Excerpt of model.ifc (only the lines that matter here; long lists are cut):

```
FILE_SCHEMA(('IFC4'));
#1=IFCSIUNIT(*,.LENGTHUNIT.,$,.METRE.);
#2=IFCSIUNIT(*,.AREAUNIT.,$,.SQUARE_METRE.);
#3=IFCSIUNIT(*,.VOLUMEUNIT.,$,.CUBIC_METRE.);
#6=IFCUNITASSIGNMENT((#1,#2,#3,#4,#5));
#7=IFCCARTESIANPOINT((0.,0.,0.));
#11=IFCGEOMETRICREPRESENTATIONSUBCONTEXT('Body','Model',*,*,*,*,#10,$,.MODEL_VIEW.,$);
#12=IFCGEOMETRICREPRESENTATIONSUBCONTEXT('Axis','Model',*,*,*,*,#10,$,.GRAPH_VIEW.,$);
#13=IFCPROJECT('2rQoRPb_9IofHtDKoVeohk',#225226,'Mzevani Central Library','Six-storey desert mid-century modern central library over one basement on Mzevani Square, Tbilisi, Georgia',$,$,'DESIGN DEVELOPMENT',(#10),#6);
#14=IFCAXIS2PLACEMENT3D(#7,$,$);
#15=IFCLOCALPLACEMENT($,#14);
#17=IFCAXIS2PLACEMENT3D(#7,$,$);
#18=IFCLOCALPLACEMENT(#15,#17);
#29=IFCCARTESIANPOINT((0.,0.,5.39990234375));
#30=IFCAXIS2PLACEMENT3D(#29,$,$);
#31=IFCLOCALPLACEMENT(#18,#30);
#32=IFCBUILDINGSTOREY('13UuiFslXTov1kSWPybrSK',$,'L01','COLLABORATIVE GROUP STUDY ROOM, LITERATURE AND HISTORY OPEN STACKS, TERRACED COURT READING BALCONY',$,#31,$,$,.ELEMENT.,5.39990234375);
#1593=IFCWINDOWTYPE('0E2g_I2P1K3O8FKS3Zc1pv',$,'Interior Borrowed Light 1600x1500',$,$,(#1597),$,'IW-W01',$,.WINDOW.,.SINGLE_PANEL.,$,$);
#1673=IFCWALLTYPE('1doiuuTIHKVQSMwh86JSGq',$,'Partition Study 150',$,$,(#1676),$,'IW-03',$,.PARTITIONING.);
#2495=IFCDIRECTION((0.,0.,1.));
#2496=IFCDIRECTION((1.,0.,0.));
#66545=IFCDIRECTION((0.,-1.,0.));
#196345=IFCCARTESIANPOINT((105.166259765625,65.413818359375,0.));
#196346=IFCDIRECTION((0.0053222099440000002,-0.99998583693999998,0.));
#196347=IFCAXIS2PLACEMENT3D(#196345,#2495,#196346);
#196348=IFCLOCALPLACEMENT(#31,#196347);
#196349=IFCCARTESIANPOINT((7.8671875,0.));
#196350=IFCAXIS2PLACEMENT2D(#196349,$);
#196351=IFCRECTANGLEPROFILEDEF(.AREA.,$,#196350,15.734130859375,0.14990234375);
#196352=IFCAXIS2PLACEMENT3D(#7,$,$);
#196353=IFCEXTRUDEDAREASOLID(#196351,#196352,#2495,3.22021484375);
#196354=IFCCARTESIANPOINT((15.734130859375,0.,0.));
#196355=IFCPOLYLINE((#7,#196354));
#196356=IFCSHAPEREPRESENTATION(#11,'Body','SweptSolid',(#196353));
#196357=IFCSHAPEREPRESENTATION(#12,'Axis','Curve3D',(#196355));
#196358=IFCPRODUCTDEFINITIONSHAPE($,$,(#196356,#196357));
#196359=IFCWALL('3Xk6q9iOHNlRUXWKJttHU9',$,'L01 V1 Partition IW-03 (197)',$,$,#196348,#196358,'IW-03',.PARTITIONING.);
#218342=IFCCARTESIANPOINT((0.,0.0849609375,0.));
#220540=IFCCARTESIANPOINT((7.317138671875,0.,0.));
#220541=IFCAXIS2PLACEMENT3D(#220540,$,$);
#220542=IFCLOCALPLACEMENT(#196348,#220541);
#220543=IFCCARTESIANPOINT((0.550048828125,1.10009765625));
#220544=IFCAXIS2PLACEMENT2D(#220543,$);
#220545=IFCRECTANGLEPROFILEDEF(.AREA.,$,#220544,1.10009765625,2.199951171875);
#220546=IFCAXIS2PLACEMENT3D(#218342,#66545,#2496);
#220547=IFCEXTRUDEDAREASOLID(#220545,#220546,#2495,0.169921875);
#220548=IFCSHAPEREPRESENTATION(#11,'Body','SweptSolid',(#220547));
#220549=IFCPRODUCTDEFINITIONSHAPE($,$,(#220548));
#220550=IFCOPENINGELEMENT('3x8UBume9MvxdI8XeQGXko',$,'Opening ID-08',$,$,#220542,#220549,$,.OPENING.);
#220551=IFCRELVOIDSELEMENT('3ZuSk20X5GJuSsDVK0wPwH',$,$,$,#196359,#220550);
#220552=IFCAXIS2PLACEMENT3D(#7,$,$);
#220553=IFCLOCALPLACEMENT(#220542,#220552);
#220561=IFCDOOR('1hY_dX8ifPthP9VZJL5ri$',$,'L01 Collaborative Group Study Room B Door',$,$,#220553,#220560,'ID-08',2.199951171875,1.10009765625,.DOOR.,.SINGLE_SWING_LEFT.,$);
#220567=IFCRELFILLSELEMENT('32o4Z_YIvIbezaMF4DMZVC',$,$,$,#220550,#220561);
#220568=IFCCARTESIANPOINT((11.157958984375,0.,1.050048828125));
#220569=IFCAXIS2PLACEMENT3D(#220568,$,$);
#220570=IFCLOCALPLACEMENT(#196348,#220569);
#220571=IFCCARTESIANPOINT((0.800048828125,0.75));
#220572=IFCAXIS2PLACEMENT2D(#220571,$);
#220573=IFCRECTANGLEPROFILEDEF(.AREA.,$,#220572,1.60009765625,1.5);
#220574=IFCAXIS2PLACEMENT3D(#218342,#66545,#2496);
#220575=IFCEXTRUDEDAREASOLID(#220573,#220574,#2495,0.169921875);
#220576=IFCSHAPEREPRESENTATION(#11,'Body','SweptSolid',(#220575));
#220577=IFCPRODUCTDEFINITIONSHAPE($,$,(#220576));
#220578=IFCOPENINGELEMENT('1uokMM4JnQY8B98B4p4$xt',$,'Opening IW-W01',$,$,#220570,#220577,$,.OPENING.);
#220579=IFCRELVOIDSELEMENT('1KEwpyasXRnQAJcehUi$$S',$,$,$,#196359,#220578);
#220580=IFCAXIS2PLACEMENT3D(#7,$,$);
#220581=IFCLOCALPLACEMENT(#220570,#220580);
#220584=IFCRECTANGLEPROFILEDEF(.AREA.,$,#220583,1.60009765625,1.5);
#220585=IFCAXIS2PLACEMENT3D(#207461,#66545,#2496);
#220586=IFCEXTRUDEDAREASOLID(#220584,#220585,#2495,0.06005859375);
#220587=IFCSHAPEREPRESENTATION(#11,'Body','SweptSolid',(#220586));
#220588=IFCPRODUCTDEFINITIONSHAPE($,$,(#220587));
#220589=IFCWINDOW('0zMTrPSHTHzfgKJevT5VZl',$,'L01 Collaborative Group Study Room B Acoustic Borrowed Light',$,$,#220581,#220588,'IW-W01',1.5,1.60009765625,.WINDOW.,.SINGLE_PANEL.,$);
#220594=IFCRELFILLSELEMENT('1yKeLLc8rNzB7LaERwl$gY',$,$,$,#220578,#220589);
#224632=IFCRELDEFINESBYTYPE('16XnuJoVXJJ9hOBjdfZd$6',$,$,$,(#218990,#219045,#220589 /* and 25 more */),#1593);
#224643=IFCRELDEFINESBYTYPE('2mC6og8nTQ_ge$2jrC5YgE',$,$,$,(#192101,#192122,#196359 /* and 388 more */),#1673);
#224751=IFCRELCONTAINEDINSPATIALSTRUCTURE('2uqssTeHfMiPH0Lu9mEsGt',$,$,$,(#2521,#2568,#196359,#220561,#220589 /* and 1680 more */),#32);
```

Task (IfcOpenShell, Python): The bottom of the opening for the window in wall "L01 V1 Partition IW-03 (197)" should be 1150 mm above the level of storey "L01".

```python
import numpy as np
import ifcopenshell
import ifcopenshell.api.geometry
import ifcopenshell.geom
import ifcopenshell.util.element
import ifcopenshell.util.placement
import ifcopenshell.util.shape
import ifcopenshell.util.unit

model = ifcopenshell.open("model.ifc")
unit_scale = ifcopenshell.util.unit.calculate_unit_scale(model)

window = model.by_guid("0zMTrPSHTHzfgKJevT5VZl")
opening = window.FillsVoids[0].RelatingOpeningElement
storey = ifcopenshell.util.element.get_container(window, ifc_class="IfcBuildingStorey")
level = ifcopenshell.util.placement.get_local_placement(storey.ObjectPlacement)[2, 3]

# The opening's origin need not be at the sill, so measure its lowest point.
shape = ifcopenshell.geom.create_shape(ifcopenshell.geom.settings(), opening)
bottom = ifcopenshell.util.shape.get_shape_bottom_elevation(shape, shape.geometry) / unit_scale
dz = level + 1.15 / unit_scale - bottom

shift = np.array([0.0, 0.0, dz])
# The window is placed relative to its opening, so it follows when the opening moves.
matrix = ifcopenshell.util.placement.get_local_placement(opening.ObjectPlacement)
matrix[:3, 3] += shift
ifcopenshell.api.geometry.edit_object_placement(
    model, product=opening, matrix=matrix, is_si=False, should_transform_children=True
)

print(f"moved by {dz * unit_scale:+.3f} m")

model.write("model_rev.ifc")
```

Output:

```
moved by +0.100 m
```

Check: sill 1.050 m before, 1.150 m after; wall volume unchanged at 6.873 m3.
